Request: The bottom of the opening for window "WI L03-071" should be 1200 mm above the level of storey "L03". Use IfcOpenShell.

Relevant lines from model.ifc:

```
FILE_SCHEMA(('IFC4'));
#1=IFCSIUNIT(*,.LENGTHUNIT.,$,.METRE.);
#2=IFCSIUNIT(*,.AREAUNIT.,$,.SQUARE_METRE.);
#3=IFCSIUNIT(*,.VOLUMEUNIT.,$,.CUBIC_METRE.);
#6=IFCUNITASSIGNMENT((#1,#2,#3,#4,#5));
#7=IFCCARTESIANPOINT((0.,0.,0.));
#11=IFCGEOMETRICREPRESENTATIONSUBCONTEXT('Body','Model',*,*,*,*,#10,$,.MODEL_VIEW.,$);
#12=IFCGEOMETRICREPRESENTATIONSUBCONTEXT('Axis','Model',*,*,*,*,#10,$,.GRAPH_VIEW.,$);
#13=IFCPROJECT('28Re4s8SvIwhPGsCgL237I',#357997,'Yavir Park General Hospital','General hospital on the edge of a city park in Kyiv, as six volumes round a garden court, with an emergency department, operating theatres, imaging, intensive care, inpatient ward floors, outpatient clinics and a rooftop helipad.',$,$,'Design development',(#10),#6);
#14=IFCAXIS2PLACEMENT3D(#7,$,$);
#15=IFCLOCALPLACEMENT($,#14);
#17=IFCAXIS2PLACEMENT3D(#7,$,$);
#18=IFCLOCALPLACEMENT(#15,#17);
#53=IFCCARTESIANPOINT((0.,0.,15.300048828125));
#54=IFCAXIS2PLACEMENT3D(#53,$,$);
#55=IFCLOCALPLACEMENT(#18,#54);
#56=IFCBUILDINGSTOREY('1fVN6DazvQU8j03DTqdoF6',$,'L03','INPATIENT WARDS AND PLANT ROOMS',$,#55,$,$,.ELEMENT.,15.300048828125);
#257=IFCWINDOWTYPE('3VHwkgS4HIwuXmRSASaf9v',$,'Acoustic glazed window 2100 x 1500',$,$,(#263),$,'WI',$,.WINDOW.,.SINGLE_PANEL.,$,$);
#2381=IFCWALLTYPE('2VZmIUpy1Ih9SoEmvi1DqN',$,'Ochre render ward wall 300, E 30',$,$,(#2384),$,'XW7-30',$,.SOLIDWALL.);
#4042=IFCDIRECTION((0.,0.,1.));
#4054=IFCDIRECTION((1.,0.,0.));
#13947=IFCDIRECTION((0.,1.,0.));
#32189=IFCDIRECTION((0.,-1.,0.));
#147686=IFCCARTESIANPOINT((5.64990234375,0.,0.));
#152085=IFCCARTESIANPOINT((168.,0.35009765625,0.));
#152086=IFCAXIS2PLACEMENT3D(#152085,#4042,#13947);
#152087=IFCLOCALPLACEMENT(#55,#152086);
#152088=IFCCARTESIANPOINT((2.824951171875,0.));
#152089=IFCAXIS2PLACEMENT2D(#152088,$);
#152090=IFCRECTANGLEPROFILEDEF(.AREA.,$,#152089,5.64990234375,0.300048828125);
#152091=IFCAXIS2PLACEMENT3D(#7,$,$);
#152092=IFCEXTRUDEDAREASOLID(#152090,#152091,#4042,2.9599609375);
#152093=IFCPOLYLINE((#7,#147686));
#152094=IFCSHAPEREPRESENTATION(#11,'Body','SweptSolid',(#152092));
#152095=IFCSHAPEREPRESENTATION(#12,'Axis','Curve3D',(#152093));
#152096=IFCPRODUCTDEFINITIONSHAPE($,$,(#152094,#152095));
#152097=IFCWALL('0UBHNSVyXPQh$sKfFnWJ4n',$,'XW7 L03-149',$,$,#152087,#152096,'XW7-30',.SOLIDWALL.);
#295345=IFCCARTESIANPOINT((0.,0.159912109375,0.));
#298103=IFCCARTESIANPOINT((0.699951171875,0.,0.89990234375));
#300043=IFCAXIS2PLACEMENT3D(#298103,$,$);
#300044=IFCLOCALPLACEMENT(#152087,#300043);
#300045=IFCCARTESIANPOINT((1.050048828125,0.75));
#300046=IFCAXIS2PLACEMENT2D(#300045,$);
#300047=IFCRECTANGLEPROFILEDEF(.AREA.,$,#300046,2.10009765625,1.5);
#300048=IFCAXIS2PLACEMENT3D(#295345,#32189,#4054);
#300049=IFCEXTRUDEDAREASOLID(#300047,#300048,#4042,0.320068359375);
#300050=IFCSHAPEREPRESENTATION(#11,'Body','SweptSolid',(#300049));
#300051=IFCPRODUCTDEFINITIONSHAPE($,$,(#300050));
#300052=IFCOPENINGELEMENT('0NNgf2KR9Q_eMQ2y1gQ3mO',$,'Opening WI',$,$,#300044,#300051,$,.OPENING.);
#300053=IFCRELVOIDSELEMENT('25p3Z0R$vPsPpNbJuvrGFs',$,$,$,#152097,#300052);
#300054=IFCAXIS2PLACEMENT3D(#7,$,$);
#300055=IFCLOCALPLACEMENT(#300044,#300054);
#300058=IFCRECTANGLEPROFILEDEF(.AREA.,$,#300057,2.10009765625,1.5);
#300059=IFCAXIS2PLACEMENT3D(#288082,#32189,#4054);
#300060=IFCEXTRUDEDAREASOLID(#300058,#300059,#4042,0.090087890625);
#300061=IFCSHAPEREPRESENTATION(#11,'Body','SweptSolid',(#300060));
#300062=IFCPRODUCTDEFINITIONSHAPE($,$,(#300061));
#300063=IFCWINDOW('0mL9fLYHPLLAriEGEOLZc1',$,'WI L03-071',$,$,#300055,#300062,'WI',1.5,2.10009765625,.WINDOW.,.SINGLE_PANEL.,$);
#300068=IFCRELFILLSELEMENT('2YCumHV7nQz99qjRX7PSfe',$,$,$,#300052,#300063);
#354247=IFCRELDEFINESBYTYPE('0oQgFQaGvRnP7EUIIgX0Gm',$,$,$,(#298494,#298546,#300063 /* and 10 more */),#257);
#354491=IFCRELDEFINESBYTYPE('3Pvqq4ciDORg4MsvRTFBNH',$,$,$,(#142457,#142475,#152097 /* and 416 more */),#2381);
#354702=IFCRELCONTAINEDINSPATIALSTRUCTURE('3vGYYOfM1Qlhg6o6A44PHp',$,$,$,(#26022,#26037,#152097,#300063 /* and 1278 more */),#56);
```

```python
import numpy as np
import ifcopenshell
import ifcopenshell.api.geometry
import ifcopenshell.geom
import ifcopenshell.util.element
import ifcopenshell.util.placement
import ifcopenshell.util.shape
import ifcopenshell.util.unit

model = ifcopenshell.open("model.ifc")
unit_scale = ifcopenshell.util.unit.calculate_unit_scale(model)

window = model.by_guid("0mL9fLYHPLLAriEGEOLZc1")
opening = window.FillsVoids[0].RelatingOpeningElement
storey = ifcopenshell.util.element.get_container(window, ifc_class="IfcBuildingStorey")
level = ifcopenshell.util.placement.get_local_placement(storey.ObjectPlacement)[2, 3]

# The opening's origin need not be at the sill, so measure its lowest point.
shape = ifcopenshell.geom.create_shape(ifcopenshell.geom.settings(), opening)
bottom = ifcopenshell.util.shape.get_shape_bottom_elevation(shape, shape.geometry) / unit_scale
dz = level + 1.2 - bottom

shift = np.array([0.0, 0.0, dz])
# The window is placed relative to its opening, so it follows when the opening moves.
matrix = ifcopenshell.util.placement.get_local_placement(opening.ObjectPlacement)
matrix[:3, 3] += shift
ifcopenshell.api.geometry.edit_object_placement(
    model, product=opening, matrix=matrix, is_si=False, should_transform_children=True
)

print(f"moved by {dz * unit_scale:+.3f} m")

model.write("model_rev.ifc")
```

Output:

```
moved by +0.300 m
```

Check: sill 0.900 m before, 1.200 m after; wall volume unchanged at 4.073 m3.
